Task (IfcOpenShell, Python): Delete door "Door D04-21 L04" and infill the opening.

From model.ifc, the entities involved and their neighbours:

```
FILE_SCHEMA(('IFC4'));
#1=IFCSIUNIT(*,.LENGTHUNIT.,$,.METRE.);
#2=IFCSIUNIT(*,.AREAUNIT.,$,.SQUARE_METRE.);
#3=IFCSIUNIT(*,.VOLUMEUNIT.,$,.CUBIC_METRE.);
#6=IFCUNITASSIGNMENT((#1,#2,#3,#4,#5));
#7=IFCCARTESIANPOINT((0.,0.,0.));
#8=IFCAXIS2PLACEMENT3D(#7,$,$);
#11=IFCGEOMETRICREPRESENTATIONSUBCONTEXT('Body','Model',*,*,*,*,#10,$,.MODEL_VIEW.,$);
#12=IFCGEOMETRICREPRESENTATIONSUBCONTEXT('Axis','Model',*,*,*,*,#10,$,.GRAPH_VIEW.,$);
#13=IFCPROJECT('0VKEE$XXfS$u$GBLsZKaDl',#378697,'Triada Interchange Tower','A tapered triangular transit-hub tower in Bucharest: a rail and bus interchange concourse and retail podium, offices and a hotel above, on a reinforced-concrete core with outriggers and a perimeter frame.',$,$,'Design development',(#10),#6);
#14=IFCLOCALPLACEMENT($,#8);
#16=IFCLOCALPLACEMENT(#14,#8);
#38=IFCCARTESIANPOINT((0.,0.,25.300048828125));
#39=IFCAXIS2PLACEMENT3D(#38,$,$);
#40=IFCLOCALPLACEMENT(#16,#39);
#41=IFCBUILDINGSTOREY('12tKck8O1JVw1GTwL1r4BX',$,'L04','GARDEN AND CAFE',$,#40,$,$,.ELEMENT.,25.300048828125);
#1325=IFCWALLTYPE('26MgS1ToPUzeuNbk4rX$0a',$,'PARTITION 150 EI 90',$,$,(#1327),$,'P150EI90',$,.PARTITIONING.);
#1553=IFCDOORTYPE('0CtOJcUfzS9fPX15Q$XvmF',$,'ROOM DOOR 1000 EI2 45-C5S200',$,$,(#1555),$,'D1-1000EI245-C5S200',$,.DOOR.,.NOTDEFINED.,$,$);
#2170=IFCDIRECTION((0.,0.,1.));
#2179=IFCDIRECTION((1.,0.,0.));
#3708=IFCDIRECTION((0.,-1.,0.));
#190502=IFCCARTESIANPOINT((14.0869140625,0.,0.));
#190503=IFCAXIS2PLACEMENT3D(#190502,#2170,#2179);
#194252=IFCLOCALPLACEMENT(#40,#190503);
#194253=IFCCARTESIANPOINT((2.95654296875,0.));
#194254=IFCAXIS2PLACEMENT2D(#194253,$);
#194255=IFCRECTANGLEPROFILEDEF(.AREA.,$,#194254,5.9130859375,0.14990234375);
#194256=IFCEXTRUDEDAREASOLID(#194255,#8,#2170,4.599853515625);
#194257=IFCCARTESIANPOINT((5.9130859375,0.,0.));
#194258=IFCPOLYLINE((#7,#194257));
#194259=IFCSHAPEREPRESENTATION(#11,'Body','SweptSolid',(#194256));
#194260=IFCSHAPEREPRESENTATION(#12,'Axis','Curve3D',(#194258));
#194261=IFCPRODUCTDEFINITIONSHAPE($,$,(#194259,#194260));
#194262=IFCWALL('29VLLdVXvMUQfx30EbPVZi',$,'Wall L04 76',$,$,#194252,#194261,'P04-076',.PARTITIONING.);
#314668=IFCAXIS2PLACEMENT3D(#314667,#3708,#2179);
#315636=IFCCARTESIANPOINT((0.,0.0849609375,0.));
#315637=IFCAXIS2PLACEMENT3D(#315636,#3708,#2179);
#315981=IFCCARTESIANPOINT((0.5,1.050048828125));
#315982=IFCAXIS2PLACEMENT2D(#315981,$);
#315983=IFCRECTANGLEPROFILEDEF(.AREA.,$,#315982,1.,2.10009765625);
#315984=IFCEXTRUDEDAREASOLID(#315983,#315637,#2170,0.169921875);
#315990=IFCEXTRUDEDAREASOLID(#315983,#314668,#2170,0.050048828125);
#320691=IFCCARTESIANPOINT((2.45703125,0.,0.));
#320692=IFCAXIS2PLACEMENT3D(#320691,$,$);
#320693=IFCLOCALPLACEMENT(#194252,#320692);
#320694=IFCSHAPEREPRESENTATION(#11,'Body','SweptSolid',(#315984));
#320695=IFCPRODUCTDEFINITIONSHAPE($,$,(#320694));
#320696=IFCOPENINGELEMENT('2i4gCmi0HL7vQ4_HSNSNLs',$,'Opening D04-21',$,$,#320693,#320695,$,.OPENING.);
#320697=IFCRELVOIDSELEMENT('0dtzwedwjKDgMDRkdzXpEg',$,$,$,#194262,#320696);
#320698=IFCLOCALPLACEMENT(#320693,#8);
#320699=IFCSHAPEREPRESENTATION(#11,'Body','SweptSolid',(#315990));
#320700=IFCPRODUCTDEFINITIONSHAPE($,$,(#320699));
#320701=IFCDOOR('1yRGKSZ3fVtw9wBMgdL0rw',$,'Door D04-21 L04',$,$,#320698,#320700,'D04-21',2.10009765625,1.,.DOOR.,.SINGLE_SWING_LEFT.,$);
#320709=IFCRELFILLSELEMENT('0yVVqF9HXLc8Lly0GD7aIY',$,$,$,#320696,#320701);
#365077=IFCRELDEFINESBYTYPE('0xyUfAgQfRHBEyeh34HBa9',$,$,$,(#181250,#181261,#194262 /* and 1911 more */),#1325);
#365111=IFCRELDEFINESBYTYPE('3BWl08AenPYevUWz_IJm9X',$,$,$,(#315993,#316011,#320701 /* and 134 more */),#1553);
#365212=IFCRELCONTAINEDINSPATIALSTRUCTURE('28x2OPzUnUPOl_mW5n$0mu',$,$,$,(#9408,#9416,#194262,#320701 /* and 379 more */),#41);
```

```python
import ifcopenshell
import ifcopenshell.api.feature
import ifcopenshell.api.root
import ifcopenshell.geom
import ifcopenshell.util.shape

model = ifcopenshell.open("model.ifc")
settings = ifcopenshell.geom.settings()


def volume(element):
    """Net volume in cubic metres, openings subtracted."""
    shape = ifcopenshell.geom.create_shape(settings, element)
    return ifcopenshell.util.shape.get_volume(shape.geometry)


door = model.by_guid("1yRGKSZ3fVtw9wBMgdL0rw")
opening = door.FillsVoids[0].RelatingOpeningElement
wall = opening.VoidsElements[0].RelatingBuildingElement
before = volume(wall)

ifcopenshell.api.root.remove_product(model, product=door)
ifcopenshell.api.feature.remove_feature(model, feature=opening)

after = volume(wall)

print(f"wall volume {before:.3f} -> {after:.3f} m3")

model.write("model_edited.ifc")
```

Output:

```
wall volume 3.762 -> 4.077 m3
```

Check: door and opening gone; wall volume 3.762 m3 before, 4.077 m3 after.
